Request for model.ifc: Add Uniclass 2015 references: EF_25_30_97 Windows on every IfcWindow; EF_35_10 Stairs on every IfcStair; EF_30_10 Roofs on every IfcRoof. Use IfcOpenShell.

First a look at what the model holds.

```python
import ifcopenshell

model = ifcopenshell.open("model.ifc")
print(model.schema)
print("classifications:", [c.Name for c in model.by_type("IfcClassification")])
for ifc_class in ("IfcDoor", "IfcRoof", "IfcStair", "IfcWall", "IfcWindow"):
    print(ifc_class, len(model.by_type(ifc_class)))
```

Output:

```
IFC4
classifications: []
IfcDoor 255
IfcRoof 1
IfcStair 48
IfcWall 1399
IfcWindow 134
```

```python
import ifcopenshell
import ifcopenshell.api.classification

model = ifcopenshell.open("model.ifc")

system = ifcopenshell.api.classification.add_classification(model, classification="Uniclass 2015")

codes = {
    "IfcWindow": ("EF_25_30_97", "Windows"),
    "IfcStair": ("EF_35_10", "Stairs"),
    "IfcRoof": ("EF_30_10", "Roofs"),
}
for ifc_class, (code, name) in codes.items():
    products = model.by_type(ifc_class)
    ifcopenshell.api.classification.add_reference(
        model, products=products, classification=system, identification=code, name=name
    )
    print(code, len(products))

model.write("model-out.ifc")
```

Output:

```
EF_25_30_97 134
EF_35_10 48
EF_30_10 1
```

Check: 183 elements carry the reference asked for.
